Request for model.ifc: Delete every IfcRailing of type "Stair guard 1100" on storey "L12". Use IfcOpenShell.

First a look at what the model holds.

```python
import ifcopenshell
import ifcopenshell.util.element

model = ifcopenshell.open("model.ifc")
print(model.schema)
storey = next(s for s in model.by_type("IfcBuildingStorey") if s.Name == "L12")
railings = [e for e in ifcopenshell.util.element.get_decomposition(storey) if e.is_a("IfcRailing")]
seen = {}
for e in railings:
    element_type = ifcopenshell.util.element.get_type(e)
    name = element_type.Name if element_type not in (None, e) else None
    seen[name] = seen.get(name, 0) + 1
for name, count in sorted(seen.items(), key=str):
    print(count, "x", name)
```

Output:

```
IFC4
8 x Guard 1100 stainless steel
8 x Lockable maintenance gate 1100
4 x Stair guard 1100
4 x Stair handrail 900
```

```python
import ifcopenshell
import ifcopenshell.api.root
import ifcopenshell.util.element

model = ifcopenshell.open("model.ifc")

storey = next(s for s in model.by_type("IfcBuildingStorey") if s.Name == "L12")
railings = [e for e in ifcopenshell.util.element.get_decomposition(storey) if e.is_a("IfcRailing")]
targets = [e for e in railings if (t := ifcopenshell.util.element.get_type(e)) not in (None, e) and t.Name == "Stair guard 1100"]

for e in targets:
    ifcopenshell.api.root.remove_product(model, product=e)
print(len(targets), "removed")

model.write("model_updated.ifc")
```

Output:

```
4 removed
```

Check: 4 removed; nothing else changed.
